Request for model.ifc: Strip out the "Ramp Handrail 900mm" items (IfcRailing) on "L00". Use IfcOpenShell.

First a look at what the model holds.

```python
import ifcopenshell
import ifcopenshell.util.element

model = ifcopenshell.open("model.ifc")
print(model.schema)
storey = next(s for s in model.by_type("IfcBuildingStorey") if s.Name == "L00")
railings = [e for e in ifcopenshell.util.element.get_decomposition(storey) if e.is_a("IfcRailing")]
seen = {}
for e in railings:
    element_type = ifcopenshell.util.element.get_type(e)
    name = element_type.Name if element_type not in (None, e) else None
    seen[name] = seen.get(name, 0) + 1
for name, count in sorted(seen.items(), key=str):
    print(count, "x", name)
```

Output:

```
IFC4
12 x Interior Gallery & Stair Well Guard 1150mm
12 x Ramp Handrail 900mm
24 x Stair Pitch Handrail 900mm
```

```python
import ifcopenshell
import ifcopenshell.api.root
import ifcopenshell.util.element

model = ifcopenshell.open("model.ifc")

storey = next(s for s in model.by_type("IfcBuildingStorey") if s.Name == "L00")
railings = [e for e in ifcopenshell.util.element.get_decomposition(storey) if e.is_a("IfcRailing")]
targets = [e for e in railings if (t := ifcopenshell.util.element.get_type(e)) not in (None, e) and t.Name == "Ramp Handrail 900mm"]

for e in targets:
    ifcopenshell.api.root.remove_product(model, product=e)
print(len(targets), "removed")

model.write("model_rev.ifc")
```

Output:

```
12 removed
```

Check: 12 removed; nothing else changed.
